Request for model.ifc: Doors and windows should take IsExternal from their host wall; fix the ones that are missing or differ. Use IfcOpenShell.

First a look at what the model holds.

```python
import ifcopenshell
import ifcopenshell.util.element

model = ifcopenshell.open("model.ifc")
print(model.schema)
seen = {}
for e in model.by_type("IfcDoor") + model.by_type("IfcWindow"):
    if not e.FillsVoids:
        continue
    host = e.FillsVoids[0].RelatingOpeningElement.VoidsElements[0].RelatingBuildingElement
    own = ifcopenshell.util.element.get_pset(e, f"Pset_{e.is_a()[3:].removesuffix('StandardCase')}Common", "IsExternal")
    wall = ifcopenshell.util.element.get_pset(host, "Pset_WallCommon", "IsExternal")
    seen[e.is_a(), own, wall] = seen.get((e.is_a(), own, wall), 0) + 1
for (cls, own, wall), count in sorted(seen.items(), key=str):
    print(count, cls, "IsExternal:", own, "| host wall:", wall)
```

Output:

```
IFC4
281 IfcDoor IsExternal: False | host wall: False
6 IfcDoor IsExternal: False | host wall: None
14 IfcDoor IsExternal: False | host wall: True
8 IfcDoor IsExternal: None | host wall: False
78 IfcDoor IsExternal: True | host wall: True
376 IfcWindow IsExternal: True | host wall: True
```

```python
import ifcopenshell
import ifcopenshell.api.pset
import ifcopenshell.util.element

model = ifcopenshell.open("model.ifc")

count = 0
for ifc_class, pset_name in (("IfcDoor", "Pset_DoorCommon"), ("IfcWindow", "Pset_WindowCommon")):
    for e in model.by_type(ifc_class):
        if not e.FillsVoids:
            continue
        host = e.FillsVoids[0].RelatingOpeningElement.VoidsElements[0].RelatingBuildingElement
        external = ifcopenshell.util.element.get_pset(host, "Pset_WallCommon", "IsExternal")
        if external is None or ifcopenshell.util.element.get_pset(e, pset_name, "IsExternal") == external:
            continue
        pset = ifcopenshell.api.pset.add_pset(model, product=e, name=pset_name)
        ifcopenshell.api.pset.edit_pset(model, pset=pset, properties={"IsExternal": external})
        count += 1

print(count, "updated")

model.write("model-out.ifc")
```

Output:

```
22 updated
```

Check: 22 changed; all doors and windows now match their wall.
